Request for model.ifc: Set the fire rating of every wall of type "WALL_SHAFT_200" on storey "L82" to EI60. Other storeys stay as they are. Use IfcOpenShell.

First a look at what the model holds.

```python
import ifcopenshell
import ifcopenshell.util.element

model = ifcopenshell.open("model.ifc")
print(model.schema)
storey = next(s for s in model.by_type("IfcBuildingStorey") if s.Name == "L82")
walls = [e for e in ifcopenshell.util.element.get_decomposition(storey) if e.is_a("IfcWall")]
seen = {}
for e in walls:
    element_type = ifcopenshell.util.element.get_type(e)
    key = (element_type.Name if element_type != e and element_type else None, ifcopenshell.util.element.get_pset(e, "Pset_WallCommon", "FireRating"))
    seen[key] = seen.get(key, 0) + 1
for (name, value), count in sorted(seen.items(), key=str):
    print(count, "x", name, "|", value)
```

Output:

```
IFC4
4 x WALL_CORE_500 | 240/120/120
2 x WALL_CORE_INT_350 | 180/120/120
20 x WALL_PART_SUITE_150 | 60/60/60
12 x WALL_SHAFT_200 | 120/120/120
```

```python
import ifcopenshell
import ifcopenshell.api.pset
import ifcopenshell.util.element

model = ifcopenshell.open("model.ifc")

storey = next(s for s in model.by_type("IfcBuildingStorey") if s.Name == "L82")
walls = [e for e in ifcopenshell.util.element.get_decomposition(storey) if e.is_a("IfcWall")]

count = 0
for e in walls:
    element_type = ifcopenshell.util.element.get_type(e)
    if element_type in (None, e) or element_type.Name != "WALL_SHAFT_200":
        continue
    found = ifcopenshell.util.element.get_pset(e, "Pset_WallCommon", should_inherit=False)
    if found:
        pset = model.by_id(found["id"])
        if len(ifcopenshell.util.element.get_elements_by_pset(pset)) > 1:
            pset = ifcopenshell.api.pset.unshare_pset(model, products=[e], pset=pset)[0]
    else:
        pset = ifcopenshell.api.pset.add_pset(model, product=e, name="Pset_WallCommon")
    ifcopenshell.api.pset.edit_pset(model, pset=pset, properties={"FireRating": "EI60"})
    count += 1

print(count, "walls updated")

model.write("model_edited.ifc")
```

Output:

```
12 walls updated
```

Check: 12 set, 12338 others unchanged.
